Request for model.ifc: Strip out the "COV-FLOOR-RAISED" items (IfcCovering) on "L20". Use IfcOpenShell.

First a look at what the model holds.

```python
import ifcopenshell
import ifcopenshell.util.element

model = ifcopenshell.open("model.ifc")
print(model.schema)
storey = next(s for s in model.by_type("IfcBuildingStorey") if s.Name == "L20")
coverings = [e for e in ifcopenshell.util.element.get_decomposition(storey) if e.is_a("IfcCovering")]
seen = {}
for e in coverings:
    element_type = ifcopenshell.util.element.get_type(e)
    name = element_type.Name if element_type not in (None, e) else None
    seen[name] = seen.get(name, 0) + 1
for name, count in sorted(seen.items(), key=str):
    print(count, "x", name)
```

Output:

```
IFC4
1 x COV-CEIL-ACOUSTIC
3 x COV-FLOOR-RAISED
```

```python
import ifcopenshell
import ifcopenshell.api.root
import ifcopenshell.util.element

model = ifcopenshell.open("model.ifc")

storey = next(s for s in model.by_type("IfcBuildingStorey") if s.Name == "L20")
coverings = [e for e in ifcopenshell.util.element.get_decomposition(storey) if e.is_a("IfcCovering")]
targets = [e for e in coverings if (t := ifcopenshell.util.element.get_type(e)) not in (None, e) and t.Name == "COV-FLOOR-RAISED"]

for e in targets:
    ifcopenshell.api.root.remove_product(model, product=e)
print(len(targets), "removed")

model.write("model_rev.ifc")
```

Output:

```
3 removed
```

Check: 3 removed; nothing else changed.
